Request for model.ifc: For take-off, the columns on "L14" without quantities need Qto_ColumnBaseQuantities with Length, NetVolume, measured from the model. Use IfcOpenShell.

First a look at what the model holds.

```python
import ifcopenshell
import ifcopenshell.util.element
import ifcopenshell.util.unit

model = ifcopenshell.open("model.ifc")
print(model.schema)
for unit_type in ("LENGTHUNIT", "AREAUNIT", "VOLUMEUNIT"):
    print(unit_type, ifcopenshell.util.unit.calculate_unit_scale(model, unit_type))
storey = next(s for s in model.by_type("IfcBuildingStorey") if s.Name == "L14")
columns = [e for e in ifcopenshell.util.element.get_decomposition(storey) if e.is_a("IfcColumn")]
for e in sorted(columns, key=lambda e: e.id()):
    print(e.id(), e.is_a(), e.Name, list(ifcopenshell.util.element.get_psets(e, qtos_only=True)), sep=" | ")
```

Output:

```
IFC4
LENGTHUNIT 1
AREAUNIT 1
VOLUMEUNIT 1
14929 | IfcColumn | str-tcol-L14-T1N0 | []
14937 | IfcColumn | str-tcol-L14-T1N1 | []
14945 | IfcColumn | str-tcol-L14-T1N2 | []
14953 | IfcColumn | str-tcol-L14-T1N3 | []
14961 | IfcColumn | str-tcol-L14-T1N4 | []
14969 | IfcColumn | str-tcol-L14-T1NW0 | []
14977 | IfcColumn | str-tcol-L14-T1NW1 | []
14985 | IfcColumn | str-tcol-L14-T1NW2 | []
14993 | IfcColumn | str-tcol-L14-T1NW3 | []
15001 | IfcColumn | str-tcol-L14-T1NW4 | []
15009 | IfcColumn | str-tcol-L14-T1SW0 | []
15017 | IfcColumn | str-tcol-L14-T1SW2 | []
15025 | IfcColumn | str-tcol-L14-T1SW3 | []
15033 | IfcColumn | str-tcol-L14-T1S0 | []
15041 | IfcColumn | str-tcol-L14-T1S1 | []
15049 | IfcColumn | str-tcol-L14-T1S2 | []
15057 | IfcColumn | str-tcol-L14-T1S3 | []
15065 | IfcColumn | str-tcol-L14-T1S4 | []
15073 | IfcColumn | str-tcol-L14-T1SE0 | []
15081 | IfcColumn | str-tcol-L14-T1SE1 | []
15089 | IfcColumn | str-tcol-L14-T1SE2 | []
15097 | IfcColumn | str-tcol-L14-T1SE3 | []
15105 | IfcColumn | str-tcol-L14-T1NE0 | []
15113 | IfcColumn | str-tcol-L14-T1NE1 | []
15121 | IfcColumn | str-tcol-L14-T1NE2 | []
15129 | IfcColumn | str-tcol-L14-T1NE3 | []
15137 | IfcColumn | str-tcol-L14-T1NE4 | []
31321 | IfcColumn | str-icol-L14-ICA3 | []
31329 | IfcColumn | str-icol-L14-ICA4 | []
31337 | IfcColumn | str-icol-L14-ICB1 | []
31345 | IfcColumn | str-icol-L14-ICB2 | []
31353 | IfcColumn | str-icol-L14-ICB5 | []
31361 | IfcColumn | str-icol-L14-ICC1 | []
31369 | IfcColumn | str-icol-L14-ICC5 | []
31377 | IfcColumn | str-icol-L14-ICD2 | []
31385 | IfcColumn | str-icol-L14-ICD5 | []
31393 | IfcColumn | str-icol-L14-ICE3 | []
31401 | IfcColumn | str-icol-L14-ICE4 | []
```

```python
import ifcopenshell
import ifcopenshell.api.pset
import ifcopenshell.geom
import ifcopenshell.util.element
import ifcopenshell.util.shape
import ifcopenshell.util.unit

model = ifcopenshell.open("model.ifc")
unit_scale = ifcopenshell.util.unit.calculate_unit_scale(model)
volume_scale = ifcopenshell.util.unit.calculate_unit_scale(model, "VOLUMEUNIT")
settings = ifcopenshell.geom.settings()

storey = next(s for s in model.by_type("IfcBuildingStorey") if s.Name == "L14")
columns = [e for e in ifcopenshell.util.element.get_decomposition(storey) if e.is_a("IfcColumn")]

for e in sorted(columns, key=lambda e: e.id()):
    if ifcopenshell.util.element.get_psets(e, qtos_only=True, should_inherit=False):
        continue
    # Geometry comes back in metres, in the element's own axes.
    shape = ifcopenshell.geom.create_shape(settings, e)
    values = {
        "Length": ifcopenshell.util.shape.get_z(shape.geometry) / unit_scale,
        "NetVolume": ifcopenshell.util.shape.get_volume(shape.geometry) / volume_scale,
    }
    qto = ifcopenshell.api.pset.add_qto(model, product=e, name="Qto_ColumnBaseQuantities")
    ifcopenshell.api.pset.edit_qto(model, qto=qto, properties=values)
    print(e.id(), {k: round(v, 3) for k, v in values.items()})

model.write("model-out.ifc")
```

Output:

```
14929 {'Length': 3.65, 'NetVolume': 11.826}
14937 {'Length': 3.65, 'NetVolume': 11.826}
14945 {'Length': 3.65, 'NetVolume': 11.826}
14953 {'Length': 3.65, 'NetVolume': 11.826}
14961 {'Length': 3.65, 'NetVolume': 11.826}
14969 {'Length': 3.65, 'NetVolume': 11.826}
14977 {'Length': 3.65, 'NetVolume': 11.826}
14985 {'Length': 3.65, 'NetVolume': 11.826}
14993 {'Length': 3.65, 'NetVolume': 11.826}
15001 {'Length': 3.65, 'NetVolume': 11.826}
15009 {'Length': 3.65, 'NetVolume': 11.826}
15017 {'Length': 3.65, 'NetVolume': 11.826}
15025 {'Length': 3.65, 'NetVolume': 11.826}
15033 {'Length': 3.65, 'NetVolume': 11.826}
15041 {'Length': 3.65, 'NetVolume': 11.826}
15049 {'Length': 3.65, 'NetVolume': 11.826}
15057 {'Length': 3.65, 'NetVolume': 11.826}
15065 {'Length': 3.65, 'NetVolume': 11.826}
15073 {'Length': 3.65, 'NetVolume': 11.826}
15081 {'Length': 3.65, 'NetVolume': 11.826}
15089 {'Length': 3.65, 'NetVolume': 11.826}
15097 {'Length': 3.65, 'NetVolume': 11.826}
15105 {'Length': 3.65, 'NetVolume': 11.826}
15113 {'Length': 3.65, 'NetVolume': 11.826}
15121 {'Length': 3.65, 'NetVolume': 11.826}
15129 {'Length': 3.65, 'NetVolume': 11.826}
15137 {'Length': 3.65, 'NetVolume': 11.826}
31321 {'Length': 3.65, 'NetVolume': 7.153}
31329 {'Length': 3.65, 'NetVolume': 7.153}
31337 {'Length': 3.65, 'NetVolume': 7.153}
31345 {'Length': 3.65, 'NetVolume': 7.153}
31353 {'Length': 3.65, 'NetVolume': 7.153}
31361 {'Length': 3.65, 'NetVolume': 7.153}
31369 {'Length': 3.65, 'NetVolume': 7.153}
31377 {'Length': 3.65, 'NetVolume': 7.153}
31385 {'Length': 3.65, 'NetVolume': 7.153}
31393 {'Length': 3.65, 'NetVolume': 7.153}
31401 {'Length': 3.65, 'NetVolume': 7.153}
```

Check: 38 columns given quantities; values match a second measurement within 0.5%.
